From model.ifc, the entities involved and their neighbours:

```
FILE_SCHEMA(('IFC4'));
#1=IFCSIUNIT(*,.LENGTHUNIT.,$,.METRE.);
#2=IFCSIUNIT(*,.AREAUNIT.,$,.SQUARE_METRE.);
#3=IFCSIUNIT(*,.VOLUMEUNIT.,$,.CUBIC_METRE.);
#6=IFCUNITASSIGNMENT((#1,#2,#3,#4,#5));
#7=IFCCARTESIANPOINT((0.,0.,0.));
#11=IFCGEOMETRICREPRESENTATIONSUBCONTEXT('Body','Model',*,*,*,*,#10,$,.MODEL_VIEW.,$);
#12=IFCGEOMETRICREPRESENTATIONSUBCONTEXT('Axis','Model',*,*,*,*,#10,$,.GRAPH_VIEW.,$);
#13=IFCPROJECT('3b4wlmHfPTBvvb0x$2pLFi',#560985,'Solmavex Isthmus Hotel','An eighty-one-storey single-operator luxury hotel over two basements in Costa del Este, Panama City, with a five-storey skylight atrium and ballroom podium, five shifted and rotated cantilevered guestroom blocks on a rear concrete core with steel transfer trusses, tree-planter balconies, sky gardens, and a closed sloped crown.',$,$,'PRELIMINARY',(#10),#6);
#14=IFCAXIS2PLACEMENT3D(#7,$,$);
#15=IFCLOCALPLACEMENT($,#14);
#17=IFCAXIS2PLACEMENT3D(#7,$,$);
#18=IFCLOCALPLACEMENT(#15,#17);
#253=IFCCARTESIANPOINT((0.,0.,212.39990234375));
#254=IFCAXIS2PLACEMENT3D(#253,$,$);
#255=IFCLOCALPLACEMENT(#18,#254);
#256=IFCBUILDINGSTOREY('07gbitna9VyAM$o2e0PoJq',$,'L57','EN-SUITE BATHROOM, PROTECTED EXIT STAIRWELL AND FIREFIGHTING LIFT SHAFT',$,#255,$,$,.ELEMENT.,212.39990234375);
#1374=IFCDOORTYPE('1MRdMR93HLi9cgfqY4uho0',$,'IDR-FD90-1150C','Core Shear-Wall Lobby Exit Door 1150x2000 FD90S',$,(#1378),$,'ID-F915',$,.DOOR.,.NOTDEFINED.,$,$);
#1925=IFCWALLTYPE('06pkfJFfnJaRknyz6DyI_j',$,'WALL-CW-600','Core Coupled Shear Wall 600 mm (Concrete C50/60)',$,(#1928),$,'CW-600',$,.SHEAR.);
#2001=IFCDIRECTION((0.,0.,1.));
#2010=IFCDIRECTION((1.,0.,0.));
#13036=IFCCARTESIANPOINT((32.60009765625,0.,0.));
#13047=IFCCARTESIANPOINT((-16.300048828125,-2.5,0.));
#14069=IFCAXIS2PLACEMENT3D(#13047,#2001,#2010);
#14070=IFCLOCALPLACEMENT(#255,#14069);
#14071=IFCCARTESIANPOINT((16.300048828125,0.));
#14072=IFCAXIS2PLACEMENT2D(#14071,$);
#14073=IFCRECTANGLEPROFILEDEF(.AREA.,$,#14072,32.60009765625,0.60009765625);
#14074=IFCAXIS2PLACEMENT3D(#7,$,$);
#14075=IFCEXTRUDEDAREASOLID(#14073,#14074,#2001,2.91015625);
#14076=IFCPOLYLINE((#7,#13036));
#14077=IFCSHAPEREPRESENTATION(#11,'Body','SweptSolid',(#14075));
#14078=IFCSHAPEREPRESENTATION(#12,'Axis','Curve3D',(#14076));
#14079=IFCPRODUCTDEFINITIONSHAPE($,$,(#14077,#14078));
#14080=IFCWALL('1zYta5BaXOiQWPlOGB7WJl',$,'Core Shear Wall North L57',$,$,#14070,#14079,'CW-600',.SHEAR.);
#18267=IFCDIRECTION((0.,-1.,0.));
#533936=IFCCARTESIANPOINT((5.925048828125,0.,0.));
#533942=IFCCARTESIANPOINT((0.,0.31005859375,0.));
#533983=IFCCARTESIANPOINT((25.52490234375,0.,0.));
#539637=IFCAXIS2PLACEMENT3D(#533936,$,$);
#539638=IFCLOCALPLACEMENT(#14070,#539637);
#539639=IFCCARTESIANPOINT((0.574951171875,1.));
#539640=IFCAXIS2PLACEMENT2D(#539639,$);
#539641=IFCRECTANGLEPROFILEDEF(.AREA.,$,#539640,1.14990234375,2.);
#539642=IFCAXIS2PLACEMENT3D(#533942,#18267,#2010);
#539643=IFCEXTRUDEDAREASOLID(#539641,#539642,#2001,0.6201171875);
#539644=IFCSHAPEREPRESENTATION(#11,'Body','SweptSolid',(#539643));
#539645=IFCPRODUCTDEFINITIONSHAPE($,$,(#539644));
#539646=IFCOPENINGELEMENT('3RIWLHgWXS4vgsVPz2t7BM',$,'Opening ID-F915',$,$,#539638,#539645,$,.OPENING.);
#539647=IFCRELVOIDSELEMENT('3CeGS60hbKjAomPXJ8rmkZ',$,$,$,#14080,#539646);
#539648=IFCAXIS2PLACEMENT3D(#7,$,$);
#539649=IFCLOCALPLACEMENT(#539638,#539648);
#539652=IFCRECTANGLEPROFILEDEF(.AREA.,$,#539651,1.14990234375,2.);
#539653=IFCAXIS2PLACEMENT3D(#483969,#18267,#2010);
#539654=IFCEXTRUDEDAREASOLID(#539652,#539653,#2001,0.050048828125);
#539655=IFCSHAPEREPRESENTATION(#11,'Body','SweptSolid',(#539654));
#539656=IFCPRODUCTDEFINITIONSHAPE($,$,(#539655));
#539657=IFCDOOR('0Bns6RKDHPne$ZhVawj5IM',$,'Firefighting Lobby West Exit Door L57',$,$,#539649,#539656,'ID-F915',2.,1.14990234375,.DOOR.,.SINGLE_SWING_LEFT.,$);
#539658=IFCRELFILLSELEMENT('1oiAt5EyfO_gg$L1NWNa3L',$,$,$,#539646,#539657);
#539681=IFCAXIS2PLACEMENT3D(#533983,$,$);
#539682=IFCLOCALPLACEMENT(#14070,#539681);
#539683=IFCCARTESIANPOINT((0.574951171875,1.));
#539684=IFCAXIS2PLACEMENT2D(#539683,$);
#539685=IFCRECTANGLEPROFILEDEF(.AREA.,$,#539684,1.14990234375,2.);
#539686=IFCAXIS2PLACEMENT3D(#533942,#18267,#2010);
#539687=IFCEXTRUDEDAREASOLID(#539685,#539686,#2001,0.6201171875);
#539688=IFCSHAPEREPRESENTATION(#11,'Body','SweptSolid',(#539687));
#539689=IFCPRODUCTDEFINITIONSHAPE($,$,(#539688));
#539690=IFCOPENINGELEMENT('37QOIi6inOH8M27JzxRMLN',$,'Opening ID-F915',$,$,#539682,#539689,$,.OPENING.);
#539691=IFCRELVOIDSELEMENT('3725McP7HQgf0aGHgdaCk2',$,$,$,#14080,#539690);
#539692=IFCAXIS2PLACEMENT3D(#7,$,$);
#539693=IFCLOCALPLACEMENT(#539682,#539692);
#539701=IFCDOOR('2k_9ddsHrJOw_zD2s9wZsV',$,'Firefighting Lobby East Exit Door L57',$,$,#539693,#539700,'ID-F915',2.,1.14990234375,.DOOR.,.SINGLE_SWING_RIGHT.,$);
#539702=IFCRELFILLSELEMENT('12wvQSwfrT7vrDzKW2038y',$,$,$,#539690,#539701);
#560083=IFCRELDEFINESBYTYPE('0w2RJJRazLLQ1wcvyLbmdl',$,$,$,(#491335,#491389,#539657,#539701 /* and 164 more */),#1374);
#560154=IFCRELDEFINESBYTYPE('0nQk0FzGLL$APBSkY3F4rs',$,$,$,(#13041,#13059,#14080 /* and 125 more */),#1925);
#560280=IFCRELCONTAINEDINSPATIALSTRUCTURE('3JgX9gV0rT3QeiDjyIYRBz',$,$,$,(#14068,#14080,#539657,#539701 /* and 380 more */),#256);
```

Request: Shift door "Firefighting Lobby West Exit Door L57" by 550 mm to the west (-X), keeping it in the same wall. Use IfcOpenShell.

```python
import ifcopenshell
import ifcopenshell.api.geometry
import ifcopenshell.util.placement
import ifcopenshell.util.unit

model = ifcopenshell.open("model.ifc")
unit_scale = ifcopenshell.util.unit.calculate_unit_scale(model)

door = model.by_id(539657)
opening = door.FillsVoids[0].RelatingOpeningElement
wall = opening.VoidsElements[0].RelatingBuildingElement

wall_matrix = ifcopenshell.util.placement.get_local_placement(wall.ObjectPlacement)
shift = wall_matrix[:3, 0] * -0.55 / unit_scale
before = ifcopenshell.util.placement.get_local_placement(door.ObjectPlacement)[:3, 3].copy()

# The door is placed relative to its opening, so it follows when the opening moves.
matrix = ifcopenshell.util.placement.get_local_placement(opening.ObjectPlacement)
matrix[:3, 3] += shift
ifcopenshell.api.geometry.edit_object_placement(
    model, product=opening, matrix=matrix, is_si=False, should_transform_children=True
)

after = ifcopenshell.util.placement.get_local_placement(door.ObjectPlacement)[:3, 3]
print("door moved by", (after - before).round(3) + 0.0)

model.write("model_edited.ifc")
```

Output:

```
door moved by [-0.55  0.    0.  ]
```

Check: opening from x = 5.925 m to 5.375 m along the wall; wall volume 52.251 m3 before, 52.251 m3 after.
